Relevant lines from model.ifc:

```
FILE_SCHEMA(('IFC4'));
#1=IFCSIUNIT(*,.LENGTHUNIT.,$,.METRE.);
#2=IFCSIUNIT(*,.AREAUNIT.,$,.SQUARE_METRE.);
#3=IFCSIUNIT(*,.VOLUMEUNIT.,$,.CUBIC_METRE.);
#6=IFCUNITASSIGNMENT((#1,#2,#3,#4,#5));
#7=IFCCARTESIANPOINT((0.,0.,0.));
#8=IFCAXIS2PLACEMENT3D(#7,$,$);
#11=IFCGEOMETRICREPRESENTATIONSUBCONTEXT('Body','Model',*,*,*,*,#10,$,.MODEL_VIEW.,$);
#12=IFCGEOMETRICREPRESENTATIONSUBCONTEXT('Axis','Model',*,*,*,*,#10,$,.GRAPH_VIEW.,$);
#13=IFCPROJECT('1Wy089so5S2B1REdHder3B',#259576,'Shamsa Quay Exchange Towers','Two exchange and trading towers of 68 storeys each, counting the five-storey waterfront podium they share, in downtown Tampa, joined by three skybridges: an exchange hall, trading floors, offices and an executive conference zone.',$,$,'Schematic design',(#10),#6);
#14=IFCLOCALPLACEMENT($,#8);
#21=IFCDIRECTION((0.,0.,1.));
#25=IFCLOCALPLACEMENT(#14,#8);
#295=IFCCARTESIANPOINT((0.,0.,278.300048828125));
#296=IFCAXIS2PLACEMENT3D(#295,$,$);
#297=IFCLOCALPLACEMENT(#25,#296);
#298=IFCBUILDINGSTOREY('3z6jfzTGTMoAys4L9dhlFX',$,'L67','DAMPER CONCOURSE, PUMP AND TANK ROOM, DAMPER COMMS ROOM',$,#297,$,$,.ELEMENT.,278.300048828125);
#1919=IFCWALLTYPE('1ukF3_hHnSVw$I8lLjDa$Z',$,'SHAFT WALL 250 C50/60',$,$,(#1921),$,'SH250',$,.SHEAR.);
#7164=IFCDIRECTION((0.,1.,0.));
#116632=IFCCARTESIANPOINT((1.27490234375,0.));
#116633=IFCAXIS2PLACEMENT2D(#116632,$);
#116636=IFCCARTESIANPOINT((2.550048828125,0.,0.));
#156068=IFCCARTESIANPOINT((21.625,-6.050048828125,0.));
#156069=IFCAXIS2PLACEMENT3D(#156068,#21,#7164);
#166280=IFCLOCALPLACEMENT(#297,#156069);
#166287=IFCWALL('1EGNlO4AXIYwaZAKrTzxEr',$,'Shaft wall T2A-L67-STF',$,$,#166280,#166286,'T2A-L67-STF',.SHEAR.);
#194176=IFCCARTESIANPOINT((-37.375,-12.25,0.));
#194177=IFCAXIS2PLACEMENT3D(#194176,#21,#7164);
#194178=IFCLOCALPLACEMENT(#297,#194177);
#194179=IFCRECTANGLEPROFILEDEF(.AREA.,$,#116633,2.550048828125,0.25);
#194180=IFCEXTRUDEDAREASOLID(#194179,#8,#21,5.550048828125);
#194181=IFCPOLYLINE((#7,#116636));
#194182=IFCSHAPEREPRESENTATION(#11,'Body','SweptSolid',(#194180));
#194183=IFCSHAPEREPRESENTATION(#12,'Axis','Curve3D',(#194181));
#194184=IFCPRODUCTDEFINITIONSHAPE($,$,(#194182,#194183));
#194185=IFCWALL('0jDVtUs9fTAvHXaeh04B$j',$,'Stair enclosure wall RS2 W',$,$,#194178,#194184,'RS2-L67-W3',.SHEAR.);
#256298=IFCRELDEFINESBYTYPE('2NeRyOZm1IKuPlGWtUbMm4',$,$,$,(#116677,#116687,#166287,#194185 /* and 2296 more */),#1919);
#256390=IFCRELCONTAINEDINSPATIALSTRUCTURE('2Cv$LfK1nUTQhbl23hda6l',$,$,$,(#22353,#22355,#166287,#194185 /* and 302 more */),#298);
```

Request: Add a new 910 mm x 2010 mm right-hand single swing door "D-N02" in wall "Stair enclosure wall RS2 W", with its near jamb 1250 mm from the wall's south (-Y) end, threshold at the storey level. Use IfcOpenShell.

```python
import numpy as np
import ifcopenshell
import ifcopenshell.api.feature
import ifcopenshell.api.geometry
import ifcopenshell.api.root
import ifcopenshell.api.spatial
import ifcopenshell.geom
import ifcopenshell.util.element
import ifcopenshell.util.placement
import ifcopenshell.util.representation
import ifcopenshell.util.shape
import ifcopenshell.util.unit

model = ifcopenshell.open("model.ifc")
unit_scale = ifcopenshell.util.unit.calculate_unit_scale(model)
settings = ifcopenshell.geom.settings()


def volume(element):
    """Net volume in cubic metres, openings subtracted."""
    shape = ifcopenshell.geom.create_shape(settings, element)
    return ifcopenshell.util.shape.get_volume(shape.geometry)


wall = model.by_id(194185)
storey = ifcopenshell.util.element.get_container(wall, ifc_class="IfcBuildingStorey")
context = ifcopenshell.util.representation.get_context(model, "Model", "Body", "MODEL_VIEW")
before = volume(wall)

width, height, from_end, sill = 0.91, 2.01, 1.25, 0.0  # metres

# The wall runs along its own X axis, and the end named is its -X end.
wall_shape = ifcopenshell.geom.create_shape(settings, wall)
x, y, z = ifcopenshell.util.shape.get_vertices(wall_shape.geometry).T
start = x.min() + from_end
face, thickness = float(y.min()), float(y.max() - y.min())
wall_matrix = ifcopenshell.util.placement.get_local_placement(wall.ObjectPlacement)
level = ifcopenshell.util.placement.get_local_placement(storey.ObjectPlacement)[2, 3]


def in_wall(x, y):
    """Placement at x, y metres in the wall's axes, at sill height."""
    matrix = wall_matrix.copy()
    matrix[:, 3] = wall_matrix @ np.array([x / unit_scale, y / unit_scale, 0.0, 1.0])
    matrix[2, 3] = level + sill / unit_scale
    return matrix


# Opening: a box that overshoots both wall faces by 50 mm.
opening = ifcopenshell.api.root.create_entity(model, ifc_class="IfcOpeningElement", predefined_type="OPENING")
box = ifcopenshell.api.geometry.add_wall_representation(
    model, context=context, length=width, height=height, thickness=thickness + 0.1
)
ifcopenshell.api.geometry.assign_representation(model, product=opening, representation=box)
ifcopenshell.api.geometry.edit_object_placement(model, product=opening, matrix=in_wall(start, face - 0.05), is_si=False)
ifcopenshell.api.feature.add_feature(model, feature=opening, element=wall)

door = ifcopenshell.api.root.create_entity(model, ifc_class="IfcDoor", name="D-N02", predefined_type="DOOR")
door.OverallWidth, door.OverallHeight = width / unit_scale, height / unit_scale
door.OperationType = "SINGLE_SWING_RIGHT"
body = ifcopenshell.api.geometry.add_door_representation(
    model,
    context=context,
    overall_width=door.OverallWidth,
    overall_height=door.OverallHeight,
    operation_type="SINGLE_SWING_RIGHT",
    lining_properties={"LiningDepth": thickness / unit_scale, "ThresholdDepth": thickness / unit_scale},
)
ifcopenshell.api.geometry.assign_representation(model, product=door, representation=body)
ifcopenshell.api.spatial.assign_container(model, products=[door], relating_structure=storey)
ifcopenshell.api.feature.add_filling(model, opening=opening, element=door)

# The lining spans the wall, so the door starts at the wall face.
ifcopenshell.api.geometry.edit_object_placement(model, product=door, matrix=in_wall(start, face), is_si=False)

after = volume(wall)

print(f"wall volume {before:.3f} -> {after:.3f} m3")

model.write("model_rev.ifc")
```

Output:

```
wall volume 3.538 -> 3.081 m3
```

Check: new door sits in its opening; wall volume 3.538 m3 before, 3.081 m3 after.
